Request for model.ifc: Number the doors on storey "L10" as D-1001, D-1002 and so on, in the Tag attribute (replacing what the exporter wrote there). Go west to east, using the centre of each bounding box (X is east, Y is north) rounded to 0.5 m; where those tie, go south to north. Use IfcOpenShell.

First a look at what the model holds.

```python
import ifcopenshell
import ifcopenshell.util.element
import ifcopenshell.util.placement

model = ifcopenshell.open("model.ifc")
print(model.schema)
storey = next(s for s in model.by_type("IfcBuildingStorey") if s.Name == "L10")
doors = [e for e in ifcopenshell.util.element.get_decomposition(storey) if e.is_a("IfcDoor")]
for e in sorted(doors, key=lambda e: e.id()):
    origin = ifcopenshell.util.placement.get_local_placement(e.ObjectPlacement)[:3, 3]
    print(e.id(), e.Tag, e.Name, origin.round(2) + 0.0, sep=" | ")
```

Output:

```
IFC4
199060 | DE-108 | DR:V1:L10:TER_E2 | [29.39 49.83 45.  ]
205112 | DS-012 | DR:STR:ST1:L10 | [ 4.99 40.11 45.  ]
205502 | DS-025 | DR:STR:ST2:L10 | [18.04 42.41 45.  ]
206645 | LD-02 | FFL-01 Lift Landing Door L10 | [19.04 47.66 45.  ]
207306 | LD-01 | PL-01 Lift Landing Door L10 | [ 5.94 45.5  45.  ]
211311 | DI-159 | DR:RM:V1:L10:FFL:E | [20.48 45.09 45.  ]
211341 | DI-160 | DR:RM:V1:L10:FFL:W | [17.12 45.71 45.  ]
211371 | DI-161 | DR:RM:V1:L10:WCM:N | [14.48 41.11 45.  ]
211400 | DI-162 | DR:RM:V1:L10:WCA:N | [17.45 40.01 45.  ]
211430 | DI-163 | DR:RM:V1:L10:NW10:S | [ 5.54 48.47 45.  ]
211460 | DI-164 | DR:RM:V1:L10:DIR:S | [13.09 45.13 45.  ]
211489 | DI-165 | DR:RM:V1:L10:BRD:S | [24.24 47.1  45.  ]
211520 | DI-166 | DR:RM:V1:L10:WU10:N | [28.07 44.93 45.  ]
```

```python
import ifcopenshell
import ifcopenshell.geom
import ifcopenshell.util.element
import ifcopenshell.util.shape

model = ifcopenshell.open("model.ifc")
settings = ifcopenshell.geom.settings()
settings.set("use-world-coords", True)


def centre(element):
    shape = ifcopenshell.geom.create_shape(settings, element)
    return ifcopenshell.util.shape.get_bbox_centroid(shape.geometry)


storey = next(s for s in model.by_type("IfcBuildingStorey") if s.Name == "L10")
doors = [e for e in ifcopenshell.util.element.get_decomposition(storey) if e.is_a("IfcDoor")]

# Insertion points can sit at a corner or the storey origin, so sort by the geometry (in metres).
centres = {e: centre(e) for e in doors}
doors.sort(key=lambda e: (round(centres[e][0] / 0.5), centres[e][1]))

for i, e in enumerate(doors, start=1):
    number = f"D-10{i:02d}"
    e.Tag = number
    print(e.id(), number)

model.write("model_rev.ifc")
```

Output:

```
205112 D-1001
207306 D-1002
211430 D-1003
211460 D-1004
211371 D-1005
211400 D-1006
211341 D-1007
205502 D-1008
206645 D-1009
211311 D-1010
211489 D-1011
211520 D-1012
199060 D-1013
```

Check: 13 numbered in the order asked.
